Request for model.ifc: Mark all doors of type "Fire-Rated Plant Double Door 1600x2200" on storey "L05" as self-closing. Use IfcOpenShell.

First a look at what the model holds.

```python
import ifcopenshell
import ifcopenshell.util.element

model = ifcopenshell.open("model.ifc")
print(model.schema)
storey = next(s for s in model.by_type("IfcBuildingStorey") if s.Name == "L05")
doors = [e for e in ifcopenshell.util.element.get_decomposition(storey) if e.is_a("IfcDoor")]
seen = {}
for e in doors:
    element_type = ifcopenshell.util.element.get_type(e)
    key = (element_type.Name if element_type != e and element_type else None, ifcopenshell.util.element.get_pset(e, "Pset_DoorCommon", "SelfClosing"))
    seen[key] = seen.get(key, 0) + 1
for (name, value), count in sorted(seen.items(), key=str):
    print(count, "x", name, "|", value)
```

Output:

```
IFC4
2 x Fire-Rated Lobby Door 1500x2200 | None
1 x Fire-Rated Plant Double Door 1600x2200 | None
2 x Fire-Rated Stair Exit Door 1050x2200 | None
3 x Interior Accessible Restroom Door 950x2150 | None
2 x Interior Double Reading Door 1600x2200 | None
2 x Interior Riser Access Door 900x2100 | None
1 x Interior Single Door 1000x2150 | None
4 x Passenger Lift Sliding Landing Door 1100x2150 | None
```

```python
import ifcopenshell
import ifcopenshell.api.pset
import ifcopenshell.util.element

model = ifcopenshell.open("model.ifc")

storey = next(s for s in model.by_type("IfcBuildingStorey") if s.Name == "L05")
doors = [e for e in ifcopenshell.util.element.get_decomposition(storey) if e.is_a("IfcDoor")]

count = 0
for e in doors:
    element_type = ifcopenshell.util.element.get_type(e)
    if element_type in (None, e) or element_type.Name != "Fire-Rated Plant Double Door 1600x2200":
        continue
    # add_pset returns the element's existing set when there is one.
    pset = ifcopenshell.api.pset.add_pset(model, product=e, name="Pset_DoorCommon")
    ifcopenshell.api.pset.edit_pset(model, pset=pset, properties={"SelfClosing": True})
    count += 1

print(count, "doors updated")

model.write("model-out.ifc")
```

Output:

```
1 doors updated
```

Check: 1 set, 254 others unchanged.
